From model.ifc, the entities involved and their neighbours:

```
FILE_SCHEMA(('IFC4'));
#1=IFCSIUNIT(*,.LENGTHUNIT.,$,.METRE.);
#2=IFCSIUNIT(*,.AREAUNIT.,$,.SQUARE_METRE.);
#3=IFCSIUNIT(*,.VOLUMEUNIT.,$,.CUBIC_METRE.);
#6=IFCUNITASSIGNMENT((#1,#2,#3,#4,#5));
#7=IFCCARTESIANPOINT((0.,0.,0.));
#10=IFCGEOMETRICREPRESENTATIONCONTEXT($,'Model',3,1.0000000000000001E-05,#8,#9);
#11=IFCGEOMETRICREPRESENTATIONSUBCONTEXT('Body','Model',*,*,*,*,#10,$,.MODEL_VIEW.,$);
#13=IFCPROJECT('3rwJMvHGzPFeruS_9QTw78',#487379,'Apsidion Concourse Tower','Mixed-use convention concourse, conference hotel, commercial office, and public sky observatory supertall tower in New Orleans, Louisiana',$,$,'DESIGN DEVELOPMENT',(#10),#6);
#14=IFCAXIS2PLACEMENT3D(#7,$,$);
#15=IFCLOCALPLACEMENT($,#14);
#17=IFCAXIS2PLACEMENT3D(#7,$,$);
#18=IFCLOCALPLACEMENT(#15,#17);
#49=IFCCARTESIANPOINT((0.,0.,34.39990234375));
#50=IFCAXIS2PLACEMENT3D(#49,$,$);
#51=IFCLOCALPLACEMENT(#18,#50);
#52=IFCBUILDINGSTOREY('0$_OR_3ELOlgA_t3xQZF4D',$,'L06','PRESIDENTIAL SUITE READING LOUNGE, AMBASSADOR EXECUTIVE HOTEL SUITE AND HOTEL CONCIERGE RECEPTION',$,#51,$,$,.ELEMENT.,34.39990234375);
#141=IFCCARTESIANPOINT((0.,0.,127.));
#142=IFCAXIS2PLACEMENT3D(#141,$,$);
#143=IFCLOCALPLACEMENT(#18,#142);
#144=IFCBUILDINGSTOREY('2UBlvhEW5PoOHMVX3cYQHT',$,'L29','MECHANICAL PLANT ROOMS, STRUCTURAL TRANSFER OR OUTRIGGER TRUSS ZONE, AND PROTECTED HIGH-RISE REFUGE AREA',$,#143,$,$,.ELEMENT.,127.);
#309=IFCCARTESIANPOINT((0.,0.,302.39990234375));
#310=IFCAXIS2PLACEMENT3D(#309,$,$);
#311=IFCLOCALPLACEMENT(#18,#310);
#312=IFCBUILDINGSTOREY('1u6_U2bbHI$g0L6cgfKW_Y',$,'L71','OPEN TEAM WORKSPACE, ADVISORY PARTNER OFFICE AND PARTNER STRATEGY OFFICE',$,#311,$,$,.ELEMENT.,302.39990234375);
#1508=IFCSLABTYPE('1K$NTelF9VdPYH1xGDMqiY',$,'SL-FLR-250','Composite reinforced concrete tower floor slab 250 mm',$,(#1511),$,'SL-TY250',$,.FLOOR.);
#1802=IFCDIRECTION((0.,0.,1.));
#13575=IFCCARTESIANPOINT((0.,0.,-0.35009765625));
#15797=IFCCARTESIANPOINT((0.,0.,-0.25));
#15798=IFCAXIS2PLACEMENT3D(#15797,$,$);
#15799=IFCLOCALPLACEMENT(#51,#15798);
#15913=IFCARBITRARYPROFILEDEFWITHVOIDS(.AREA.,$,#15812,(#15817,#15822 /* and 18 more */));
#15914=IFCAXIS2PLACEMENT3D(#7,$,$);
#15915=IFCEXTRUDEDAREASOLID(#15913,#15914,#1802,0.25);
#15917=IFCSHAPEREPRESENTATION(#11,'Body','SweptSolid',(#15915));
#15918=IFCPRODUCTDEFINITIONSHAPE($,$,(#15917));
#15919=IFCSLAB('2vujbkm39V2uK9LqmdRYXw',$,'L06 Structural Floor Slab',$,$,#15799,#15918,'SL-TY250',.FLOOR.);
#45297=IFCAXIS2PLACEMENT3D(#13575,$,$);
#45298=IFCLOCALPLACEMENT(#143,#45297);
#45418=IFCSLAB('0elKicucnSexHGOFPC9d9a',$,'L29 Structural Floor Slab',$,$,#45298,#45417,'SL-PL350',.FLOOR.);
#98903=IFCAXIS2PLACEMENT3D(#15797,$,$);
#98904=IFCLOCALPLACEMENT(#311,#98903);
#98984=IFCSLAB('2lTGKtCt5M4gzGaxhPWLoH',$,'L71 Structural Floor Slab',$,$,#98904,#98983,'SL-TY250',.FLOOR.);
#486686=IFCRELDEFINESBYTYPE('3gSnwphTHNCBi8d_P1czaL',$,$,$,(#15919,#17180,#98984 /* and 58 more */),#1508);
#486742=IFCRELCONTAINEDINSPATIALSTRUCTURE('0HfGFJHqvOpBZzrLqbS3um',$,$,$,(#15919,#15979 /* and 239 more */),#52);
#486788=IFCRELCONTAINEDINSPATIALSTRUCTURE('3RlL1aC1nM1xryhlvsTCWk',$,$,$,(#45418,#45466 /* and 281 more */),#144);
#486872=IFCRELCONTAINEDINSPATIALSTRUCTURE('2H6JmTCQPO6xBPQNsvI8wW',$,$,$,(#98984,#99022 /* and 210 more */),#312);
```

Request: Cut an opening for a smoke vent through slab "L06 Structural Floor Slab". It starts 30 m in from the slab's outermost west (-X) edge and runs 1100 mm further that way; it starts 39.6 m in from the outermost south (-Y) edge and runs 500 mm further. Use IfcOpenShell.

```python
import numpy as np
import ifcopenshell
import ifcopenshell.api.feature
import ifcopenshell.api.geometry
import ifcopenshell.api.root
import ifcopenshell.geom
import ifcopenshell.util.placement
import ifcopenshell.util.representation
import ifcopenshell.util.shape
import ifcopenshell.util.unit

model = ifcopenshell.open("model.ifc")
unit_scale = ifcopenshell.util.unit.calculate_unit_scale(model)
settings = ifcopenshell.geom.settings()


def volume(element):
    """Net volume in cubic metres, openings subtracted."""
    shape = ifcopenshell.geom.create_shape(settings, element)
    return ifcopenshell.util.shape.get_volume(shape.geometry)


slab = model.by_guid("2vujbkm39V2uK9LqmdRYXw")
before = volume(slab)

# Extent in the slab's own axes, in metres. The edges named are its -X and -Y sides.
slab_shape = ifcopenshell.geom.create_shape(settings, slab)
vertices = ifcopenshell.util.shape.get_vertices(slab_shape.geometry)
x_min, y_min, bottom = vertices.min(axis=0)
top = vertices[:, 2].max()

opening = ifcopenshell.api.root.create_entity(model, ifc_class="IfcOpeningElement", name="Smoke vent opening", predefined_type="OPENING")
context = ifcopenshell.util.representation.get_context(model, "Model", "Body", "MODEL_VIEW")
width, depth = 1.1, 0.5
outline = [(0.0, 0.0), (width, 0.0), (width, depth), (0.0, depth), (0.0, 0.0)]
# Overshoot both faces by 50 mm so the cut is clean.
shape = ifcopenshell.api.geometry.add_slab_representation(
    model, context=context, depth=top - bottom + 0.1, polyline=outline
)
ifcopenshell.api.geometry.assign_representation(model, product=opening, representation=shape)

matrix = ifcopenshell.util.placement.get_local_placement(slab.ObjectPlacement)
matrix[:, 3] = matrix @ np.append(np.array([x_min + 30, y_min + 39.6, bottom - 0.05]) / unit_scale, 1.0)
ifcopenshell.api.geometry.edit_object_placement(model, product=opening, matrix=matrix, is_si=False)
ifcopenshell.api.feature.add_feature(model, feature=opening, element=slab)

after = volume(slab)

print(f"slab volume {before:.3f} -> {after:.3f} m3")

model.write("model_rev.ifc")
```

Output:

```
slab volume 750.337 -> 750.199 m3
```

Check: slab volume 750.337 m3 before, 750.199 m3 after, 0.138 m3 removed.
